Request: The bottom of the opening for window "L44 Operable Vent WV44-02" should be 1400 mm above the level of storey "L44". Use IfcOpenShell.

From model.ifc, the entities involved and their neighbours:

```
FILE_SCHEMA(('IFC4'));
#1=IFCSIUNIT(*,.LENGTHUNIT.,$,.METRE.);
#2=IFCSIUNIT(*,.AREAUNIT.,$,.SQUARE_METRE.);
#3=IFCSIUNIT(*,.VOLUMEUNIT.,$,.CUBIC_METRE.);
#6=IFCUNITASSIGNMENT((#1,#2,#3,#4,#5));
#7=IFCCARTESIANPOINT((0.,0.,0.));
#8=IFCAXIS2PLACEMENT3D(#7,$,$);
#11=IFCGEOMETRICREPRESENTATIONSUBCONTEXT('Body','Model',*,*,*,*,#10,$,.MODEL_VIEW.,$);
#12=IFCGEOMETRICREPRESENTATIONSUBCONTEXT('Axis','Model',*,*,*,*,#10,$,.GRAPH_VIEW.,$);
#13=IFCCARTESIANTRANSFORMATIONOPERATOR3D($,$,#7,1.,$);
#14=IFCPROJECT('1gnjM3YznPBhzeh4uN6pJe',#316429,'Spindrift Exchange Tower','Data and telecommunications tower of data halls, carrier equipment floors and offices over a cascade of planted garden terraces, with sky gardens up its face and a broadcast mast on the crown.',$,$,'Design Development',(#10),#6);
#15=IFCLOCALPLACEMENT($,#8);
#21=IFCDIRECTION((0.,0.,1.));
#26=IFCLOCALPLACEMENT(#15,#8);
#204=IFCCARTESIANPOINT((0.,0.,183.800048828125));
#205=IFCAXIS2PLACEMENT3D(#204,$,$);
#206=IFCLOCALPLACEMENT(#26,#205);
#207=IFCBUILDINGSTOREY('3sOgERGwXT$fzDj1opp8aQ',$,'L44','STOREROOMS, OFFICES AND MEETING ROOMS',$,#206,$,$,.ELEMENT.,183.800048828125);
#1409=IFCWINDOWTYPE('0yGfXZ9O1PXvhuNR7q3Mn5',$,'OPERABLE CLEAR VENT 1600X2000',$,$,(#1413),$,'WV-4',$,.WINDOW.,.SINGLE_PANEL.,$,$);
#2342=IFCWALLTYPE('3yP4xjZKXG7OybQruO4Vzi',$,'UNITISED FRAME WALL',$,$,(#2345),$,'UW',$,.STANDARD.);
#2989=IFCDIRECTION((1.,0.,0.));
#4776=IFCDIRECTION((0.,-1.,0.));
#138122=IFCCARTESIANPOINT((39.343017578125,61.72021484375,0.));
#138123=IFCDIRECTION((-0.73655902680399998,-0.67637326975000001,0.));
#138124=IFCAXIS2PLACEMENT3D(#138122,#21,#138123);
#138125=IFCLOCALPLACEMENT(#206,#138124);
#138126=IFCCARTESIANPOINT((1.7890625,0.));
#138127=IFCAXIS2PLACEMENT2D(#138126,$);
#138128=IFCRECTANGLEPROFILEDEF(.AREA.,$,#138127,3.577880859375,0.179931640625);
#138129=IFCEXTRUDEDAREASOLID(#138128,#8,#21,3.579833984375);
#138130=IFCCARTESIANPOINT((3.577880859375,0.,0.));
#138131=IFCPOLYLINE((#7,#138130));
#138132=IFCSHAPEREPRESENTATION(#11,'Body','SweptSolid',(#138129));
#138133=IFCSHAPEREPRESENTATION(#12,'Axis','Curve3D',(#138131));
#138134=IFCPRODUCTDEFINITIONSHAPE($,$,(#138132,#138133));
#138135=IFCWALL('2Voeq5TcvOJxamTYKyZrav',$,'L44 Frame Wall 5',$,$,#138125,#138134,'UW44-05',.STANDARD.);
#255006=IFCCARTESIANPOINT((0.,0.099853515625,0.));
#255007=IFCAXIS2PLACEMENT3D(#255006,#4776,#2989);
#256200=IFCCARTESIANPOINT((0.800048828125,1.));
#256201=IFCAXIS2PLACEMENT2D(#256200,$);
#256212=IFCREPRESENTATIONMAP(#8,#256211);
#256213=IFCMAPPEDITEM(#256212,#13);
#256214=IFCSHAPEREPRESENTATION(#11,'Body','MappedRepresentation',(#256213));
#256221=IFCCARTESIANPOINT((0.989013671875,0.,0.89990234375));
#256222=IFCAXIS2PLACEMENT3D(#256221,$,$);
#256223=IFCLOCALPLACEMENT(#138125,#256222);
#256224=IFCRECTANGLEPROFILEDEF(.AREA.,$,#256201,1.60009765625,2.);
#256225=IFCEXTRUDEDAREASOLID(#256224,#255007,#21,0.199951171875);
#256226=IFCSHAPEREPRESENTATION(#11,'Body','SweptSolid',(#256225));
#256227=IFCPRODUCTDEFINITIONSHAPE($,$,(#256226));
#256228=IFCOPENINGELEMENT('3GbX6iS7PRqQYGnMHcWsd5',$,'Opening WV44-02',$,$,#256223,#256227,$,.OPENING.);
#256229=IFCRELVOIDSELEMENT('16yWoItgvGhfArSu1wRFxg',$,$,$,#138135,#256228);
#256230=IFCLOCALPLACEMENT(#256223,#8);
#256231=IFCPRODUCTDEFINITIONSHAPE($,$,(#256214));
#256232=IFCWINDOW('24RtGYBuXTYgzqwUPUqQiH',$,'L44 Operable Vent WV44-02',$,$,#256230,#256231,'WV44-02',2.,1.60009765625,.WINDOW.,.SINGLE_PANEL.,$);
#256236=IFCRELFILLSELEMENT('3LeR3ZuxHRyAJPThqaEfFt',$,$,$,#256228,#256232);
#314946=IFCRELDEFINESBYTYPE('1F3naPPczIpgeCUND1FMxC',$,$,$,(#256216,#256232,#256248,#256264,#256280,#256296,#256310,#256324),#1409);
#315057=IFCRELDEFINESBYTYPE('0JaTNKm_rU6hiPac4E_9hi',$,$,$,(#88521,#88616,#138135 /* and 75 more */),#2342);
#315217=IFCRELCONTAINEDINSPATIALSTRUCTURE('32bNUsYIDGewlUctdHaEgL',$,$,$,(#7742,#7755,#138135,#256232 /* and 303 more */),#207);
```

```python
import numpy as np
import ifcopenshell
import ifcopenshell.api.geometry
import ifcopenshell.geom
import ifcopenshell.util.element
import ifcopenshell.util.placement
import ifcopenshell.util.shape
import ifcopenshell.util.unit

model = ifcopenshell.open("model.ifc")
unit_scale = ifcopenshell.util.unit.calculate_unit_scale(model)

window = model.by_id(256232)
opening = window.FillsVoids[0].RelatingOpeningElement
storey = ifcopenshell.util.element.get_container(window, ifc_class="IfcBuildingStorey")
level = ifcopenshell.util.placement.get_local_placement(storey.ObjectPlacement)[2, 3]

# The opening's origin need not be at the sill, so measure its lowest point.
shape = ifcopenshell.geom.create_shape(ifcopenshell.geom.settings(), opening)
bottom = ifcopenshell.util.shape.get_shape_bottom_elevation(shape, shape.geometry) / unit_scale
dz = level + 1.4 - bottom

shift = np.array([0.0, 0.0, dz])
# The window is placed relative to its opening, so it follows when the opening moves.
matrix = ifcopenshell.util.placement.get_local_placement(opening.ObjectPlacement)
matrix[:3, 3] += shift
ifcopenshell.api.geometry.edit_object_placement(
    model, product=opening, matrix=matrix, is_si=False, should_transform_children=True
)

print(f"moved by {dz * unit_scale:+.3f} m")

model.write("model_updated.ifc")
```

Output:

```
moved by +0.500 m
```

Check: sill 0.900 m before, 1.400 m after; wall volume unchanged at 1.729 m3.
